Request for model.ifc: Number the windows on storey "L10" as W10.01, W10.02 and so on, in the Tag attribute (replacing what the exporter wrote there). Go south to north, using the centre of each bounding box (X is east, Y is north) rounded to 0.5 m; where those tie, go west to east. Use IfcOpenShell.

First a look at what the model holds.

```python
import ifcopenshell
import ifcopenshell.util.element
import ifcopenshell.util.placement

model = ifcopenshell.open("model.ifc")
print(model.schema)
storey = next(s for s in model.by_type("IfcBuildingStorey") if s.Name == "L10")
windows = [e for e in ifcopenshell.util.element.get_decomposition(storey) if e.is_a("IfcWindow")]
for e in sorted(windows, key=lambda e: e.id()):
    origin = ifcopenshell.util.placement.get_local_placement(e.ObjectPlacement)[:3, 3]
    print(e.id(), e.Tag, e.Name, origin.round(2) + 0.0, sep=" | ")
```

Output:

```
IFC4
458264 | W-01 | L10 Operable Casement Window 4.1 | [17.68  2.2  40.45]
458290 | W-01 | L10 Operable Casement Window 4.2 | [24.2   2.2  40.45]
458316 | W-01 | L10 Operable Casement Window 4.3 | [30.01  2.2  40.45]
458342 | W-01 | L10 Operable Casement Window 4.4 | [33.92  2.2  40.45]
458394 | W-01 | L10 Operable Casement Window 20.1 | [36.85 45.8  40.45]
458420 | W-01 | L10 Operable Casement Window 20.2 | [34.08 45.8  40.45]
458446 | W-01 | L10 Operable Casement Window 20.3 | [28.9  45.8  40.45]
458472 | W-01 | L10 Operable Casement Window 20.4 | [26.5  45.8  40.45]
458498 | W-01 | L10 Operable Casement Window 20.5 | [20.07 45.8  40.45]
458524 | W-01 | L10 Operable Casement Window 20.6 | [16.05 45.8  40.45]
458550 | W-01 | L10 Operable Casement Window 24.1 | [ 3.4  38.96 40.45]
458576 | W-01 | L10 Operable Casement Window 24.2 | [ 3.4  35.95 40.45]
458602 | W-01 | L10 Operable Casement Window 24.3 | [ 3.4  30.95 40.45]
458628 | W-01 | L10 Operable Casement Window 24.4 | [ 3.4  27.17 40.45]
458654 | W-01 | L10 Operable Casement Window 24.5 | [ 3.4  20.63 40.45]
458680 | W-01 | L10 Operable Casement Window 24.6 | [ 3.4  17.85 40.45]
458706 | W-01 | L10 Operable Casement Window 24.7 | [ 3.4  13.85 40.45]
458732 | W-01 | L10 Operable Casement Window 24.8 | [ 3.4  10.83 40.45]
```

```python
import ifcopenshell
import ifcopenshell.geom
import ifcopenshell.util.element
import ifcopenshell.util.shape

model = ifcopenshell.open("model.ifc")
settings = ifcopenshell.geom.settings()
settings.set("use-world-coords", True)


def centre(element):
    shape = ifcopenshell.geom.create_shape(settings, element)
    return ifcopenshell.util.shape.get_bbox_centroid(shape.geometry)


storey = next(s for s in model.by_type("IfcBuildingStorey") if s.Name == "L10")
windows = [e for e in ifcopenshell.util.element.get_decomposition(storey) if e.is_a("IfcWindow")]

# Insertion points can sit at a corner or the storey origin, so sort by the geometry (in metres).
centres = {e: centre(e) for e in windows}
windows.sort(key=lambda e: (round(centres[e][1] / 0.5), centres[e][0]))

for i, e in enumerate(windows, start=1):
    number = f"W10.{i:02d}"
    e.Tag = number
    print(e.id(), number)

model.write("model-out.ifc")
```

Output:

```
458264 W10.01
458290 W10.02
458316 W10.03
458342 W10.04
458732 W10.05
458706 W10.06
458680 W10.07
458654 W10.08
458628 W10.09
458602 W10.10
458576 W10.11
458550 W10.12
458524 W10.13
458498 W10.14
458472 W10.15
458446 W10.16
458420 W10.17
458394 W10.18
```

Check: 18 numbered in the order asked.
